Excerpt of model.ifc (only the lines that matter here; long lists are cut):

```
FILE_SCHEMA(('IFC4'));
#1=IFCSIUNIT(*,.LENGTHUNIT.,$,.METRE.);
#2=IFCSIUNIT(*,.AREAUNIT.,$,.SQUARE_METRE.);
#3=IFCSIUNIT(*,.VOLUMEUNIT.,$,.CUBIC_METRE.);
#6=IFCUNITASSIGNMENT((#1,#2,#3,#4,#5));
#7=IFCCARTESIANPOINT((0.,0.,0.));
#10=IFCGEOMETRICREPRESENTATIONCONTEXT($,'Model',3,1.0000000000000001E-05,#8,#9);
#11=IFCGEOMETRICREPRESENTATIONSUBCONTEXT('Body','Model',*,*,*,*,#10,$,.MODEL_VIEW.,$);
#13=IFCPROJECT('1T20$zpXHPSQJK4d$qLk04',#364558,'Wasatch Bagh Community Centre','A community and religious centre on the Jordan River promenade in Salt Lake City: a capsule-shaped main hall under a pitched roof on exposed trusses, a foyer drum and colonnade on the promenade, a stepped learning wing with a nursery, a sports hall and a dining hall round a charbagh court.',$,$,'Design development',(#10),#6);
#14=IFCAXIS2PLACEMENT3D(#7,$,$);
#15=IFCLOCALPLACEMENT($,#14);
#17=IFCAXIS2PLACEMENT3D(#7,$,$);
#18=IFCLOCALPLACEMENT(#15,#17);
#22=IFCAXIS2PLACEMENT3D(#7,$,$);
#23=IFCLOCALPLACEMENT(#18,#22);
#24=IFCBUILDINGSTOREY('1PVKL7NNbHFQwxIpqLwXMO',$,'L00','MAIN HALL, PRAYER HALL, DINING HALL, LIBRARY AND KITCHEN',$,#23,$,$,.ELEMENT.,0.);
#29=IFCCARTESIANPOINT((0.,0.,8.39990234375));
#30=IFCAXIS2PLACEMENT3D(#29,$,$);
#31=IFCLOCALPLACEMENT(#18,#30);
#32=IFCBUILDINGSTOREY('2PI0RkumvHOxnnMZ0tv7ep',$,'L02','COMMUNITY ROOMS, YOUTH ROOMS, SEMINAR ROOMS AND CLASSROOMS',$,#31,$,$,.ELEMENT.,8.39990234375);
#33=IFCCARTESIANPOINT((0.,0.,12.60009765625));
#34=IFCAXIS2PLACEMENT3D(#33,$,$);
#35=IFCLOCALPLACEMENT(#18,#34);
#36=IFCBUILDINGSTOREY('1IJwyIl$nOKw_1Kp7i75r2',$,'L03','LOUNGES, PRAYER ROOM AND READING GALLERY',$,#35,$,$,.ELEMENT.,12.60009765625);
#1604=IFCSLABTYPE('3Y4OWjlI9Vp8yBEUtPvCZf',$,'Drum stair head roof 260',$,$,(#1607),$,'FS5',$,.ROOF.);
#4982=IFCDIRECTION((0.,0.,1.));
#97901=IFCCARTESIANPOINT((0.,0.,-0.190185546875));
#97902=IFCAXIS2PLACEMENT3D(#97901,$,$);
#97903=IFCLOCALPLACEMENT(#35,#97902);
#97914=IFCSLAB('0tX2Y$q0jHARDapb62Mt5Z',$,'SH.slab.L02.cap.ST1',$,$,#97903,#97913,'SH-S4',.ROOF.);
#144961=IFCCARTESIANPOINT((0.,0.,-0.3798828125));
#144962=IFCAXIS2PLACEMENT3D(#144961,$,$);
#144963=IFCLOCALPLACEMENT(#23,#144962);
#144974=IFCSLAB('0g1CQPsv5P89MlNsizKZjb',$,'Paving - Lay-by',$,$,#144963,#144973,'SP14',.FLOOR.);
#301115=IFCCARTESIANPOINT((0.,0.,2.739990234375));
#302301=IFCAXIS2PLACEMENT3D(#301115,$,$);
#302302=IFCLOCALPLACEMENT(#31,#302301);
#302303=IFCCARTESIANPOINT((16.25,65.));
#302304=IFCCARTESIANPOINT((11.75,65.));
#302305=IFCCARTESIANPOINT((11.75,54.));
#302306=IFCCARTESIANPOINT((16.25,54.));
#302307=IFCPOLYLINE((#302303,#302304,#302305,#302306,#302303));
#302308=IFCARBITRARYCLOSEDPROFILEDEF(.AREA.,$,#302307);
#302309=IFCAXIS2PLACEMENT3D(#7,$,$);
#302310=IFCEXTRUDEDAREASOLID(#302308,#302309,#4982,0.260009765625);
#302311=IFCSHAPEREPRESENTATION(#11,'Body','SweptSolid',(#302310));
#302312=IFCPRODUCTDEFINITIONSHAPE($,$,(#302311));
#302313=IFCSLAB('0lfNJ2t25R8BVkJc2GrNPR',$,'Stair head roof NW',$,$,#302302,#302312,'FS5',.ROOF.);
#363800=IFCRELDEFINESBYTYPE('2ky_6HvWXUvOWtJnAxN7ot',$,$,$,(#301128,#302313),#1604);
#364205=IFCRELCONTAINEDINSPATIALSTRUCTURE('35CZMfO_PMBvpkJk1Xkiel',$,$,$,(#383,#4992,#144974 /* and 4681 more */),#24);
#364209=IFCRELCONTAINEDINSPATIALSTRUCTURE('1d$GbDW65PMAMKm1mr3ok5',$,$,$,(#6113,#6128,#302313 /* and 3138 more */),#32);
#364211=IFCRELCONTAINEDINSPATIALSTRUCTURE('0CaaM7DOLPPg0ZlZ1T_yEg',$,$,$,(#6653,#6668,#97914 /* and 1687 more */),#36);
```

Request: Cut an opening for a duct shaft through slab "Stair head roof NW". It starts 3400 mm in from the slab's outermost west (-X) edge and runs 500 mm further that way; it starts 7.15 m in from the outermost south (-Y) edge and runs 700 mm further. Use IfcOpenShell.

```python
import numpy as np
import ifcopenshell
import ifcopenshell.api.feature
import ifcopenshell.api.geometry
import ifcopenshell.api.root
import ifcopenshell.geom
import ifcopenshell.util.placement
import ifcopenshell.util.representation
import ifcopenshell.util.shape
import ifcopenshell.util.unit

model = ifcopenshell.open("model.ifc")
unit_scale = ifcopenshell.util.unit.calculate_unit_scale(model)
settings = ifcopenshell.geom.settings()


def volume(element):
    """Net volume in cubic metres, openings subtracted."""
    shape = ifcopenshell.geom.create_shape(settings, element)
    return ifcopenshell.util.shape.get_volume(shape.geometry)


slab = model.by_id(302313)
before = volume(slab)

# Extent in the slab's own axes, in metres. The edges named are its -X and -Y sides.
slab_shape = ifcopenshell.geom.create_shape(settings, slab)
vertices = ifcopenshell.util.shape.get_vertices(slab_shape.geometry)
x_min, y_min, bottom = vertices.min(axis=0)
top = vertices[:, 2].max()

opening = ifcopenshell.api.root.create_entity(model, ifc_class="IfcOpeningElement", name="Duct shaft opening", predefined_type="OPENING")
context = ifcopenshell.util.representation.get_context(model, "Model", "Body", "MODEL_VIEW")
width, depth = 0.5, 0.7
outline = [(0.0, 0.0), (width, 0.0), (width, depth), (0.0, depth), (0.0, 0.0)]
# Overshoot both faces by 50 mm so the cut is clean.
shape = ifcopenshell.api.geometry.add_slab_representation(
    model, context=context, depth=top - bottom + 0.1, polyline=outline
)
ifcopenshell.api.geometry.assign_representation(model, product=opening, representation=shape)

matrix = ifcopenshell.util.placement.get_local_placement(slab.ObjectPlacement)
matrix[:, 3] = matrix @ np.append(np.array([x_min + 3.4, y_min + 7.15, bottom - 0.05]) / unit_scale, 1.0)
ifcopenshell.api.geometry.edit_object_placement(model, product=opening, matrix=matrix, is_si=False)
ifcopenshell.api.feature.add_feature(model, feature=opening, element=slab)

after = volume(slab)

print(f"slab volume {before:.3f} -> {after:.3f} m3")

model.write("model_edited.ifc")
```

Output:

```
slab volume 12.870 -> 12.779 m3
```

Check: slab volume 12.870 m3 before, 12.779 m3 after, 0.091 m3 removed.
